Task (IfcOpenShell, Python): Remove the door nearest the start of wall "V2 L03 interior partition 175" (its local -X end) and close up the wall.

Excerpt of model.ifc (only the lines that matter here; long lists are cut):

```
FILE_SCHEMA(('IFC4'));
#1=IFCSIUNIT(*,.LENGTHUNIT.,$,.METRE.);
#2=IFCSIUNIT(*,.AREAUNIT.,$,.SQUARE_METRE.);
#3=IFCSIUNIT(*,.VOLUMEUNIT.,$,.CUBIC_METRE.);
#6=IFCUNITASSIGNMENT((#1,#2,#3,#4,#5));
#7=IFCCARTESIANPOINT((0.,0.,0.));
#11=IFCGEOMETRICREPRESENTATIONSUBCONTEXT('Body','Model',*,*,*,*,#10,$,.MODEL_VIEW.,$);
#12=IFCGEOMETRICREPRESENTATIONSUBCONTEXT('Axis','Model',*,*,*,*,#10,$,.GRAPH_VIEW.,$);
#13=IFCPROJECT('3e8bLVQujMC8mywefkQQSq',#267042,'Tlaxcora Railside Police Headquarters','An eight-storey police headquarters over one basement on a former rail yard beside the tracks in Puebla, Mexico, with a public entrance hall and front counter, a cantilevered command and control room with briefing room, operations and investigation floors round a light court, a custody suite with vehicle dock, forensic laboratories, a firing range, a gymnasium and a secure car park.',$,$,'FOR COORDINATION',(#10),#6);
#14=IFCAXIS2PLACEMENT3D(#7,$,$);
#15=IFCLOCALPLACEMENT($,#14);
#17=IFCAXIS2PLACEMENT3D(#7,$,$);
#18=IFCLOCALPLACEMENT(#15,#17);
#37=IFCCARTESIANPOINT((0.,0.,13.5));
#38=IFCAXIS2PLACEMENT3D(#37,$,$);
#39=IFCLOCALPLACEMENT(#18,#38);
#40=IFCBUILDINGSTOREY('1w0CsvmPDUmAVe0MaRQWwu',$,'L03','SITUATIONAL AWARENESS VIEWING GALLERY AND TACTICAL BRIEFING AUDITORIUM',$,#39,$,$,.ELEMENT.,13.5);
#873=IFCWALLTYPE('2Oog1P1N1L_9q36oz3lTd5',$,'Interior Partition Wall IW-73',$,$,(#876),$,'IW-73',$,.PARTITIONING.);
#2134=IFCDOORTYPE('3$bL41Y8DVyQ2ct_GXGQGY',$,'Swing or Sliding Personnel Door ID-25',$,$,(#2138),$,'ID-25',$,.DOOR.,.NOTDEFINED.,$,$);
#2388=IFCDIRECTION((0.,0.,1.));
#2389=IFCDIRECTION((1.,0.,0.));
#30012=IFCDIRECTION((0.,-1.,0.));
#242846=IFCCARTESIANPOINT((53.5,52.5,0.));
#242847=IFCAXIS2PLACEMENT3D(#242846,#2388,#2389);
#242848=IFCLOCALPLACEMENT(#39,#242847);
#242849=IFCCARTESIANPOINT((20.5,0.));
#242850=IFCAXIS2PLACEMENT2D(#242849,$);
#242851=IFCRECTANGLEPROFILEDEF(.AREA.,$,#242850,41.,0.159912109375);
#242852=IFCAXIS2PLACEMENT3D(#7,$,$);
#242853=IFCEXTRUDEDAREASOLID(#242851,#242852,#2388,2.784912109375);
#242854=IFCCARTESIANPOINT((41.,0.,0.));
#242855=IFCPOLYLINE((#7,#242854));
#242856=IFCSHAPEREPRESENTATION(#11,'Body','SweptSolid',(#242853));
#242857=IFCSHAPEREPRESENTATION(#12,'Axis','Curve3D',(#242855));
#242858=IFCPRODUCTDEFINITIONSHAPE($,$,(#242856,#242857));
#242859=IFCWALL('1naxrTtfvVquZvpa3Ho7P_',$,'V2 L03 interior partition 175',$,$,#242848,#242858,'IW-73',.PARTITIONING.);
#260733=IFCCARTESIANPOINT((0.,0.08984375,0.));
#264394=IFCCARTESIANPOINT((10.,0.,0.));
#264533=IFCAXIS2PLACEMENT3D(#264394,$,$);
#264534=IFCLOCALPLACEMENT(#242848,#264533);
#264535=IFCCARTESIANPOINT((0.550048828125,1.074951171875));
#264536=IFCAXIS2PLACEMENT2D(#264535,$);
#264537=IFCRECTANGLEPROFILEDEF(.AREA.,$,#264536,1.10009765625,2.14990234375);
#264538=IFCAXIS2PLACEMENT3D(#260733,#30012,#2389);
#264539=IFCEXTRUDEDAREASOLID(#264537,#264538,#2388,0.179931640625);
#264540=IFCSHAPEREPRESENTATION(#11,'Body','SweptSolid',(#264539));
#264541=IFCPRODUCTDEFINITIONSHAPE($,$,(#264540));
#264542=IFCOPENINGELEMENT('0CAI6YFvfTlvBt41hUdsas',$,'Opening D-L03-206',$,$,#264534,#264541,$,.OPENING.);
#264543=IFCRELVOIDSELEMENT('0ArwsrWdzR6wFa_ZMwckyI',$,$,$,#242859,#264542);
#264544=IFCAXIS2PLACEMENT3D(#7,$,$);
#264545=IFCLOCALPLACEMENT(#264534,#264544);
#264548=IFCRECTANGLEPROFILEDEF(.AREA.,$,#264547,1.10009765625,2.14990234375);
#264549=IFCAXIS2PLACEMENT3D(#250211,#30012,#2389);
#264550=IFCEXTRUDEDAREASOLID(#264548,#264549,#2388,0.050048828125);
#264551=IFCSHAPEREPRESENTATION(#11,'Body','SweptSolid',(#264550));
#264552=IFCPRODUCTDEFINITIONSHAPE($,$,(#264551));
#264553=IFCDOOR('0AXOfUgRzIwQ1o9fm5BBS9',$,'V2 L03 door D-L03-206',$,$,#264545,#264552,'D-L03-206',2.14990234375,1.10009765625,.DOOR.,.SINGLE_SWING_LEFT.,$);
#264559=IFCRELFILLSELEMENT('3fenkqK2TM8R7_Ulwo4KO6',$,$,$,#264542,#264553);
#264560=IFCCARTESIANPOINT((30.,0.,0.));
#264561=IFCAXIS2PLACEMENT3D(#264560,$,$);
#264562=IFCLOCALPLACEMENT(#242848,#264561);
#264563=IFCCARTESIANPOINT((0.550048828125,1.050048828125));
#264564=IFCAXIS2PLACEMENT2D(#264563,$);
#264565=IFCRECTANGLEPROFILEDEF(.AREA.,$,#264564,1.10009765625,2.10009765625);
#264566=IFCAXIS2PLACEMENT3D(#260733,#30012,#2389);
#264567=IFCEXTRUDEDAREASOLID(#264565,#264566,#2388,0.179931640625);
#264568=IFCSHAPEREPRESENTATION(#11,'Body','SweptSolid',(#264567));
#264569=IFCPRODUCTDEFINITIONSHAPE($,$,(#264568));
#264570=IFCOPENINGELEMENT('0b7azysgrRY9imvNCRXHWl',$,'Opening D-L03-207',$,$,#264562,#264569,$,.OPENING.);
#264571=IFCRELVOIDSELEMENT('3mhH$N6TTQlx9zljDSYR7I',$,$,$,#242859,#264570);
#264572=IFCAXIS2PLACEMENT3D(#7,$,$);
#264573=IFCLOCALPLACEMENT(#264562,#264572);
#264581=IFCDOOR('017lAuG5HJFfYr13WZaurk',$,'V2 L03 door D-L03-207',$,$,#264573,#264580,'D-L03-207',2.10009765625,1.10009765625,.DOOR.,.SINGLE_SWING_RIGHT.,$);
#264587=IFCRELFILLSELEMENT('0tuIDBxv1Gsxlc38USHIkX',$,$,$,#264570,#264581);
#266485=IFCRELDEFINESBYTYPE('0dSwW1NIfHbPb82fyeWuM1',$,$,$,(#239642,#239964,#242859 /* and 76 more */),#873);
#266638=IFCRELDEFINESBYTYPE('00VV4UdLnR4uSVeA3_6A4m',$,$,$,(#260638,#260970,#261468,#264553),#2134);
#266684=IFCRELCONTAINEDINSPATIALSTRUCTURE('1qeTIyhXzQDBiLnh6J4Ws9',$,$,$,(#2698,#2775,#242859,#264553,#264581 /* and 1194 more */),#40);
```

```python
import ifcopenshell
import ifcopenshell.api.feature
import ifcopenshell.api.root
import ifcopenshell.geom
import ifcopenshell.util.shape

model = ifcopenshell.open("model.ifc")
settings = ifcopenshell.geom.settings()


def volume(element):
    """Net volume in cubic metres, openings subtracted."""
    shape = ifcopenshell.geom.create_shape(settings, element)
    return ifcopenshell.util.shape.get_volume(shape.geometry)


door = model.by_guid("0AXOfUgRzIwQ1o9fm5BBS9")
opening = door.FillsVoids[0].RelatingOpeningElement
wall = opening.VoidsElements[0].RelatingBuildingElement
before = volume(wall)

ifcopenshell.api.root.remove_product(model, product=door)
ifcopenshell.api.feature.remove_feature(model, feature=opening)

after = volume(wall)

print(f"wall volume {before:.3f} -> {after:.3f} m3")

model.write("model_updated.ifc")
```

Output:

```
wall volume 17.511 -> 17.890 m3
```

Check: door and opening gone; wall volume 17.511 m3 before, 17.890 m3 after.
